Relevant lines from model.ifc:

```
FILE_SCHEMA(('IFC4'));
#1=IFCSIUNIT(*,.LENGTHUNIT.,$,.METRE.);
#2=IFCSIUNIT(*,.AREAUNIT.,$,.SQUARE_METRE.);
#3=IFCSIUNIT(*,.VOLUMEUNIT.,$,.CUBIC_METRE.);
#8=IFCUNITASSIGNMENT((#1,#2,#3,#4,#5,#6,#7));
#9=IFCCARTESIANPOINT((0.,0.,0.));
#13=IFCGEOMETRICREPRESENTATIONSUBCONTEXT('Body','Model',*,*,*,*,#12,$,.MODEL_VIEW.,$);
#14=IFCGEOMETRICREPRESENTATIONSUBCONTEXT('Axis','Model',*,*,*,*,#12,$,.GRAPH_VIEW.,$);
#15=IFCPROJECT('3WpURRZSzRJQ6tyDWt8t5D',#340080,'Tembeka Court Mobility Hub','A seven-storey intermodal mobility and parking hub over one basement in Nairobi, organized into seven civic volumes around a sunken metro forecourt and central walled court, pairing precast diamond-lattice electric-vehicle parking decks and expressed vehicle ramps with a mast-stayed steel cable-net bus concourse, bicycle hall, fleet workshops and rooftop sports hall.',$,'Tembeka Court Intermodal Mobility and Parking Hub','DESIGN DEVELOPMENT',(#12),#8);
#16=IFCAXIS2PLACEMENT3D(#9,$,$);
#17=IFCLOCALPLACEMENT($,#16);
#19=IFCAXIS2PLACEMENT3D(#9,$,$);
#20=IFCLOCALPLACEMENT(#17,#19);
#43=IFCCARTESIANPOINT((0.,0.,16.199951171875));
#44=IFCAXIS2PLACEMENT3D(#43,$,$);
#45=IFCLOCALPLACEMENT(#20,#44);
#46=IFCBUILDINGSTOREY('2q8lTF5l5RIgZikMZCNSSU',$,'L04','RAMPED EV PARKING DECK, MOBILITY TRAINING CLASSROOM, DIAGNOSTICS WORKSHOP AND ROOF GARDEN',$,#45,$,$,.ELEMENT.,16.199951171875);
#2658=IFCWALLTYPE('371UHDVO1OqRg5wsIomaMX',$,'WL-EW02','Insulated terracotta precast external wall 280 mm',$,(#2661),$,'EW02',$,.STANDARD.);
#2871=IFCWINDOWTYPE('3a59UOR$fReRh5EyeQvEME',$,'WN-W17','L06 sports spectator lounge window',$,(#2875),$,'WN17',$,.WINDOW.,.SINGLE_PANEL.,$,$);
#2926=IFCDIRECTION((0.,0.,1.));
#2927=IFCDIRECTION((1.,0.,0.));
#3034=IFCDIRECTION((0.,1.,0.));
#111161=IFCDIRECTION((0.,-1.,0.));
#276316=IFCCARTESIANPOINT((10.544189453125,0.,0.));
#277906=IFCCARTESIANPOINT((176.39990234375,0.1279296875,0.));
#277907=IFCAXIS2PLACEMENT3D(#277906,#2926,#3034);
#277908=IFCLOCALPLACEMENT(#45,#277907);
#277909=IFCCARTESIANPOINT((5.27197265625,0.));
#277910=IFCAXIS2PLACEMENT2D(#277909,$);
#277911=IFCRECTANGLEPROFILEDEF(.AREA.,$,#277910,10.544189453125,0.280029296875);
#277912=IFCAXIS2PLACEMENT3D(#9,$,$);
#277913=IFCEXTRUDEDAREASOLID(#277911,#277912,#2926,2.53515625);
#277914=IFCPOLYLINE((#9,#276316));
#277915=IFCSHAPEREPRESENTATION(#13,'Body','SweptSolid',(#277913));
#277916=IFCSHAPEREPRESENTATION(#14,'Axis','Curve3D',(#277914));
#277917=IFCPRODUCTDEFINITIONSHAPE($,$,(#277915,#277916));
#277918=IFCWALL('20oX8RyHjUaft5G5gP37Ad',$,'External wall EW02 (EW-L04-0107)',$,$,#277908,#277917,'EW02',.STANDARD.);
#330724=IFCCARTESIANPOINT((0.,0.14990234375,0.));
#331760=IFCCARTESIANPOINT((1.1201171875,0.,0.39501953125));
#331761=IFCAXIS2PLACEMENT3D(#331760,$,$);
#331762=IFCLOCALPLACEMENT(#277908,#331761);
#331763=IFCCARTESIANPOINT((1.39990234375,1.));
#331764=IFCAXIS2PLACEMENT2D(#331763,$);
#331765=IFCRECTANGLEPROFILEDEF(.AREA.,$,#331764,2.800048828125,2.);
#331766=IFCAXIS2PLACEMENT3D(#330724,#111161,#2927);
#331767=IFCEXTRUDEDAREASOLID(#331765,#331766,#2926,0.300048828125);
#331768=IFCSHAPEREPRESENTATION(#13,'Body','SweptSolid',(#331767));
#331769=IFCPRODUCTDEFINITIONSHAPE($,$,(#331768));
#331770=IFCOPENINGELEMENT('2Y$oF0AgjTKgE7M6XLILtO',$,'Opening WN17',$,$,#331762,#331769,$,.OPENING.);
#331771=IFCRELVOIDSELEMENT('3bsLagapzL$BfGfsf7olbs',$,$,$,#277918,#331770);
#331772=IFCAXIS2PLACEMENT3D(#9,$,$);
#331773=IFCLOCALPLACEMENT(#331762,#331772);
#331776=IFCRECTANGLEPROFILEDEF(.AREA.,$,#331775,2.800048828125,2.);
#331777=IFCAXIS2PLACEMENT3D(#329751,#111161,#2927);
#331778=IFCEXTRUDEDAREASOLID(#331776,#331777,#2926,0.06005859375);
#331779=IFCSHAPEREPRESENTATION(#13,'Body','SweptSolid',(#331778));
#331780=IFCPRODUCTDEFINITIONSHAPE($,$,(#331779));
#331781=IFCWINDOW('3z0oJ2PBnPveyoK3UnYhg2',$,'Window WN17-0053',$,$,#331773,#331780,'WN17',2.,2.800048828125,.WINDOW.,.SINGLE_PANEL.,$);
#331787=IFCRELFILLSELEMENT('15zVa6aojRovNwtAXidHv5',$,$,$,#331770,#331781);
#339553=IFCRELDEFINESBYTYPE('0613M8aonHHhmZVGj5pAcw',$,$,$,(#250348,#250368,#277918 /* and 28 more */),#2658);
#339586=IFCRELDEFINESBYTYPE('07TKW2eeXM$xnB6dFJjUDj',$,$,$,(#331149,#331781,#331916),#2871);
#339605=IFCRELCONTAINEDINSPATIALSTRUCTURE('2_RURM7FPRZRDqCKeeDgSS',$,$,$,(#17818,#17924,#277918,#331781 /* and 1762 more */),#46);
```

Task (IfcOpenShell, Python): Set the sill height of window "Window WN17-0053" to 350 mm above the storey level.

```python
import numpy as np
import ifcopenshell
import ifcopenshell.api.geometry
import ifcopenshell.geom
import ifcopenshell.util.element
import ifcopenshell.util.placement
import ifcopenshell.util.shape
import ifcopenshell.util.unit

model = ifcopenshell.open("model.ifc")
unit_scale = ifcopenshell.util.unit.calculate_unit_scale(model)

window = model.by_guid("3z0oJ2PBnPveyoK3UnYhg2")
opening = window.FillsVoids[0].RelatingOpeningElement
storey = ifcopenshell.util.element.get_container(window, ifc_class="IfcBuildingStorey")
level = ifcopenshell.util.placement.get_local_placement(storey.ObjectPlacement)[2, 3]

# The opening's origin need not be at the sill, so measure its lowest point.
shape = ifcopenshell.geom.create_shape(ifcopenshell.geom.settings(), opening)
bottom = ifcopenshell.util.shape.get_shape_bottom_elevation(shape, shape.geometry) / unit_scale
dz = level + 0.35 / unit_scale - bottom

shift = np.array([0.0, 0.0, dz])
# The window is placed relative to its opening, so it follows when the opening moves.
matrix = ifcopenshell.util.placement.get_local_placement(opening.ObjectPlacement)
matrix[:3, 3] += shift
ifcopenshell.api.geometry.edit_object_placement(
    model, product=opening, matrix=matrix, is_si=False, should_transform_children=True
)

print(f"moved by {dz * unit_scale:+.3f} m")

model.write("model-out.ifc")
```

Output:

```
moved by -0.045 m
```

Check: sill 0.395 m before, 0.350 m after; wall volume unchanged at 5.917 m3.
